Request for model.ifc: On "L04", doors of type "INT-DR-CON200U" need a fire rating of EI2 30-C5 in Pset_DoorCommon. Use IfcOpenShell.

First a look at what the model holds.

```python
import ifcopenshell
import ifcopenshell.util.element

model = ifcopenshell.open("model.ifc")
print(model.schema)
storey = next(s for s in model.by_type("IfcBuildingStorey") if s.Name == "L04")
doors = [e for e in ifcopenshell.util.element.get_decomposition(storey) if e.is_a("IfcDoor")]
seen = {}
for e in doors:
    element_type = ifcopenshell.util.element.get_type(e)
    key = (element_type.Name if element_type != e and element_type else None, ifcopenshell.util.element.get_pset(e, "Pset_DoorCommon", "FireRating"))
    seen[key] = seen.get(key, 0) + 1
for (name, value), count in sorted(seen.items(), key=str):
    print(count, "x", name, "|", value)
```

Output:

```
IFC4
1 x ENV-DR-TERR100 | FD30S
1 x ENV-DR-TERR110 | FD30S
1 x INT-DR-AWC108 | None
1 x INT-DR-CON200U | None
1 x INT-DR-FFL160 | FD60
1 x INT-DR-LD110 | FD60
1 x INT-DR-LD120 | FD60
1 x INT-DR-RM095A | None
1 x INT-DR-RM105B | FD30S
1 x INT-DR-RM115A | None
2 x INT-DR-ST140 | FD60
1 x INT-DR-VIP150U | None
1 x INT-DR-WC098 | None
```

```python
import ifcopenshell
import ifcopenshell.api.pset
import ifcopenshell.util.element

model = ifcopenshell.open("model.ifc")

storey = next(s for s in model.by_type("IfcBuildingStorey") if s.Name == "L04")
doors = [e for e in ifcopenshell.util.element.get_decomposition(storey) if e.is_a("IfcDoor")]

count = 0
for e in doors:
    element_type = ifcopenshell.util.element.get_type(e)
    if element_type in (None, e) or element_type.Name != "INT-DR-CON200U":
        continue
    # add_pset returns the element's existing set when there is one.
    pset = ifcopenshell.api.pset.add_pset(model, product=e, name="Pset_DoorCommon")
    ifcopenshell.api.pset.edit_pset(model, pset=pset, properties={"FireRating": "EI2 30-C5"})
    count += 1

print(count, "doors updated")

model.write("model_v2.ifc")
```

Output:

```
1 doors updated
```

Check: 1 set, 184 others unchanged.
